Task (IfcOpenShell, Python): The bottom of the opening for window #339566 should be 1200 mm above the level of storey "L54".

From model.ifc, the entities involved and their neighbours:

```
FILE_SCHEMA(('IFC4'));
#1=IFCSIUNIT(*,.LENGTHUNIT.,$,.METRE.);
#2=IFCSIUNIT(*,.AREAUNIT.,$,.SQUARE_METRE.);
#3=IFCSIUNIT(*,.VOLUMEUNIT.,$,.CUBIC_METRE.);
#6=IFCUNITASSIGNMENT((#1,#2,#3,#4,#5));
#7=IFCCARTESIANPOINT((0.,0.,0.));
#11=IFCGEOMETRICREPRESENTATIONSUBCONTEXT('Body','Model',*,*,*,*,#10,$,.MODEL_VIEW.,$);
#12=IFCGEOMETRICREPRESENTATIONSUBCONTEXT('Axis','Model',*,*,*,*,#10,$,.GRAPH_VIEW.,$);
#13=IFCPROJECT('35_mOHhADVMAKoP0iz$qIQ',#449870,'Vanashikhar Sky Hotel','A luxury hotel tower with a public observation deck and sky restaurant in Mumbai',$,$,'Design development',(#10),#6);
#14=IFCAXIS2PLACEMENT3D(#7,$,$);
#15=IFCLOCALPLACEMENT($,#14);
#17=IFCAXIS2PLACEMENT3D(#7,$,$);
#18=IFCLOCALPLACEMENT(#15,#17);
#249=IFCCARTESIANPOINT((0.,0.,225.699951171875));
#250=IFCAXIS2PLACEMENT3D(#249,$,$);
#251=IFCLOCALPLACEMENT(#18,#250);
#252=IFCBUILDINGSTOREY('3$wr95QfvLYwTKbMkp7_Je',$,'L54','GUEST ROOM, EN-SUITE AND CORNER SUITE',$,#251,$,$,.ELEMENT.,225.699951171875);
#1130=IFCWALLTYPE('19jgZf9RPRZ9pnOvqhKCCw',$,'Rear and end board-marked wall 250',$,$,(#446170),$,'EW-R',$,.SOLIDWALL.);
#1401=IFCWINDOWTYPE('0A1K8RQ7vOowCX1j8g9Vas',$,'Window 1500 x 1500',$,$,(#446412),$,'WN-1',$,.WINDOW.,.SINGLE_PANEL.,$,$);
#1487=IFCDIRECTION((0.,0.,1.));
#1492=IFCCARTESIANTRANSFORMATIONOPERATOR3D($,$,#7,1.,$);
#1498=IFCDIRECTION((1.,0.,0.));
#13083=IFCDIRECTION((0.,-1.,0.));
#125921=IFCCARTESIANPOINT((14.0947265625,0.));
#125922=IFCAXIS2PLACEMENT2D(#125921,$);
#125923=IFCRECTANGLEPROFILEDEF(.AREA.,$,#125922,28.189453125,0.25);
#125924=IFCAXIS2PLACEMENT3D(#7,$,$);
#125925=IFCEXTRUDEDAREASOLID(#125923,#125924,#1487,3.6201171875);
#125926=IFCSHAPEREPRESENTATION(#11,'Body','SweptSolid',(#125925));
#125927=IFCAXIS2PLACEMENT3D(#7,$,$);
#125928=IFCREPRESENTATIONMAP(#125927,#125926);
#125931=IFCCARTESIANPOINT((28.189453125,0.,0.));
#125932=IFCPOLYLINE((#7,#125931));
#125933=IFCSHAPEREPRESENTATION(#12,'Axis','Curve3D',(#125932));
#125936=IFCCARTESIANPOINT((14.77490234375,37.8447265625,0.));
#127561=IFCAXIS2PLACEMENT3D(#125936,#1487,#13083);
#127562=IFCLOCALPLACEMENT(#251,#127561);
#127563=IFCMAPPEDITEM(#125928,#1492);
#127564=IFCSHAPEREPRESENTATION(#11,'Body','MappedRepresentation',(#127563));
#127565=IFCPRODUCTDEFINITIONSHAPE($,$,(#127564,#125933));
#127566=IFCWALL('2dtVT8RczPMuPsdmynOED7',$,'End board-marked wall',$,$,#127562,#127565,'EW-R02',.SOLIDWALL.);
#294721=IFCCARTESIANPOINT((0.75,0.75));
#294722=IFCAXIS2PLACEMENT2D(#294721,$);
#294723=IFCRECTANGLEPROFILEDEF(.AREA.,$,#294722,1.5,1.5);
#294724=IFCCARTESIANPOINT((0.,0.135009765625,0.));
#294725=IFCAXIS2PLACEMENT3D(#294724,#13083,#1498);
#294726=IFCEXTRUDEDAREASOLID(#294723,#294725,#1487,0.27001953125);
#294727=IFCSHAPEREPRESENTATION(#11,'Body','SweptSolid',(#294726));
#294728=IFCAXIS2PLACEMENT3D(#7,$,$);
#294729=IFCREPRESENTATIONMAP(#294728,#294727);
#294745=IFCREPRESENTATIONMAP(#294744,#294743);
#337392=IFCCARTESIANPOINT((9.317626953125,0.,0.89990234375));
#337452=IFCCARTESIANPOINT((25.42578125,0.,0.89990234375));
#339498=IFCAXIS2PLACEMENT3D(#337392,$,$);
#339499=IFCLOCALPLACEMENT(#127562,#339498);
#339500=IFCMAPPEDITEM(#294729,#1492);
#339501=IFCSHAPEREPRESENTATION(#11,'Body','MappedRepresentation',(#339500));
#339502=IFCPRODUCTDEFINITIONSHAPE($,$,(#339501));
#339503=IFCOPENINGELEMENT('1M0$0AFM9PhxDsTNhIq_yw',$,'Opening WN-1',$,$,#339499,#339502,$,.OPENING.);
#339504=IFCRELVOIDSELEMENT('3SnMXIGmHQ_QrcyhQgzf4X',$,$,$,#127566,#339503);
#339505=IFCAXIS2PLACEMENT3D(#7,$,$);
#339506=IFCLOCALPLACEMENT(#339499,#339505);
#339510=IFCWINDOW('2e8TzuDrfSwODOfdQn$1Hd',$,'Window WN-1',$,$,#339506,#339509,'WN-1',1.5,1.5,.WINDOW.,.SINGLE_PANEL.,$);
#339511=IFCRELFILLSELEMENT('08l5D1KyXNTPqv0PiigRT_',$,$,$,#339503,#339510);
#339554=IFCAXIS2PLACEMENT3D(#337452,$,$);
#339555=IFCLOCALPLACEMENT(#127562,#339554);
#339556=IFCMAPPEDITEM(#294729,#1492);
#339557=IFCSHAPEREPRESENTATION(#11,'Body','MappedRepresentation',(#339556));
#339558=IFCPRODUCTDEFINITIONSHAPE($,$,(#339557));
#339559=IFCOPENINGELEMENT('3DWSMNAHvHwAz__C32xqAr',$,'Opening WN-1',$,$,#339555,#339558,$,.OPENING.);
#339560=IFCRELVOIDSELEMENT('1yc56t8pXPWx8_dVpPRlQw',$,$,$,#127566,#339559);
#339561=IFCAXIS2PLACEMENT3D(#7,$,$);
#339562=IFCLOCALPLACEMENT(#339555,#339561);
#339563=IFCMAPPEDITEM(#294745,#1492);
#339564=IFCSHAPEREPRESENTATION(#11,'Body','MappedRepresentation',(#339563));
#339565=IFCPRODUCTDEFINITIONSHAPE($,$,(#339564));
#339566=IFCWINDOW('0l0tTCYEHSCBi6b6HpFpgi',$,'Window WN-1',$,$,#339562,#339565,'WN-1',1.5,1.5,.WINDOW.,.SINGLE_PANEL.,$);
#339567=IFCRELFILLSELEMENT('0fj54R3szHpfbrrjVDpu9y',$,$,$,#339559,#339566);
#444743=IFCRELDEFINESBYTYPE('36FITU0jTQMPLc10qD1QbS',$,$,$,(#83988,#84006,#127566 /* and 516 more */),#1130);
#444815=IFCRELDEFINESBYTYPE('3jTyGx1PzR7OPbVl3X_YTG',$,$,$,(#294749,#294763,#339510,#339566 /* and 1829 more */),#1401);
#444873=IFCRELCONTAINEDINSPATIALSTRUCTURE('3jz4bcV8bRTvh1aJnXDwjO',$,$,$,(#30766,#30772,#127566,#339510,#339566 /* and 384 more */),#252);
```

```python
import numpy as np
import ifcopenshell
import ifcopenshell.api.geometry
import ifcopenshell.geom
import ifcopenshell.util.element
import ifcopenshell.util.placement
import ifcopenshell.util.shape
import ifcopenshell.util.unit

model = ifcopenshell.open("model.ifc")
unit_scale = ifcopenshell.util.unit.calculate_unit_scale(model)

window = model.by_guid("0l0tTCYEHSCBi6b6HpFpgi")
opening = window.FillsVoids[0].RelatingOpeningElement
storey = ifcopenshell.util.element.get_container(window, ifc_class="IfcBuildingStorey")
level = ifcopenshell.util.placement.get_local_placement(storey.ObjectPlacement)[2, 3]

# The opening's origin need not be at the sill, so measure its lowest point.
shape = ifcopenshell.geom.create_shape(ifcopenshell.geom.settings(), opening)
bottom = ifcopenshell.util.shape.get_shape_bottom_elevation(shape, shape.geometry) / unit_scale
dz = level + 1.2 / unit_scale - bottom

shift = np.array([0.0, 0.0, dz])
# The window is placed relative to its opening, so it follows when the opening moves.
matrix = ifcopenshell.util.placement.get_local_placement(opening.ObjectPlacement)
matrix[:3, 3] += shift
ifcopenshell.api.geometry.edit_object_placement(
    model, product=opening, matrix=matrix, is_si=False, should_transform_children=True
)

print(f"moved by {dz * unit_scale:+.3f} m")

model.write("model-out.ifc")
```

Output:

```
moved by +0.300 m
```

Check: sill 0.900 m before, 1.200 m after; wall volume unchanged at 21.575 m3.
